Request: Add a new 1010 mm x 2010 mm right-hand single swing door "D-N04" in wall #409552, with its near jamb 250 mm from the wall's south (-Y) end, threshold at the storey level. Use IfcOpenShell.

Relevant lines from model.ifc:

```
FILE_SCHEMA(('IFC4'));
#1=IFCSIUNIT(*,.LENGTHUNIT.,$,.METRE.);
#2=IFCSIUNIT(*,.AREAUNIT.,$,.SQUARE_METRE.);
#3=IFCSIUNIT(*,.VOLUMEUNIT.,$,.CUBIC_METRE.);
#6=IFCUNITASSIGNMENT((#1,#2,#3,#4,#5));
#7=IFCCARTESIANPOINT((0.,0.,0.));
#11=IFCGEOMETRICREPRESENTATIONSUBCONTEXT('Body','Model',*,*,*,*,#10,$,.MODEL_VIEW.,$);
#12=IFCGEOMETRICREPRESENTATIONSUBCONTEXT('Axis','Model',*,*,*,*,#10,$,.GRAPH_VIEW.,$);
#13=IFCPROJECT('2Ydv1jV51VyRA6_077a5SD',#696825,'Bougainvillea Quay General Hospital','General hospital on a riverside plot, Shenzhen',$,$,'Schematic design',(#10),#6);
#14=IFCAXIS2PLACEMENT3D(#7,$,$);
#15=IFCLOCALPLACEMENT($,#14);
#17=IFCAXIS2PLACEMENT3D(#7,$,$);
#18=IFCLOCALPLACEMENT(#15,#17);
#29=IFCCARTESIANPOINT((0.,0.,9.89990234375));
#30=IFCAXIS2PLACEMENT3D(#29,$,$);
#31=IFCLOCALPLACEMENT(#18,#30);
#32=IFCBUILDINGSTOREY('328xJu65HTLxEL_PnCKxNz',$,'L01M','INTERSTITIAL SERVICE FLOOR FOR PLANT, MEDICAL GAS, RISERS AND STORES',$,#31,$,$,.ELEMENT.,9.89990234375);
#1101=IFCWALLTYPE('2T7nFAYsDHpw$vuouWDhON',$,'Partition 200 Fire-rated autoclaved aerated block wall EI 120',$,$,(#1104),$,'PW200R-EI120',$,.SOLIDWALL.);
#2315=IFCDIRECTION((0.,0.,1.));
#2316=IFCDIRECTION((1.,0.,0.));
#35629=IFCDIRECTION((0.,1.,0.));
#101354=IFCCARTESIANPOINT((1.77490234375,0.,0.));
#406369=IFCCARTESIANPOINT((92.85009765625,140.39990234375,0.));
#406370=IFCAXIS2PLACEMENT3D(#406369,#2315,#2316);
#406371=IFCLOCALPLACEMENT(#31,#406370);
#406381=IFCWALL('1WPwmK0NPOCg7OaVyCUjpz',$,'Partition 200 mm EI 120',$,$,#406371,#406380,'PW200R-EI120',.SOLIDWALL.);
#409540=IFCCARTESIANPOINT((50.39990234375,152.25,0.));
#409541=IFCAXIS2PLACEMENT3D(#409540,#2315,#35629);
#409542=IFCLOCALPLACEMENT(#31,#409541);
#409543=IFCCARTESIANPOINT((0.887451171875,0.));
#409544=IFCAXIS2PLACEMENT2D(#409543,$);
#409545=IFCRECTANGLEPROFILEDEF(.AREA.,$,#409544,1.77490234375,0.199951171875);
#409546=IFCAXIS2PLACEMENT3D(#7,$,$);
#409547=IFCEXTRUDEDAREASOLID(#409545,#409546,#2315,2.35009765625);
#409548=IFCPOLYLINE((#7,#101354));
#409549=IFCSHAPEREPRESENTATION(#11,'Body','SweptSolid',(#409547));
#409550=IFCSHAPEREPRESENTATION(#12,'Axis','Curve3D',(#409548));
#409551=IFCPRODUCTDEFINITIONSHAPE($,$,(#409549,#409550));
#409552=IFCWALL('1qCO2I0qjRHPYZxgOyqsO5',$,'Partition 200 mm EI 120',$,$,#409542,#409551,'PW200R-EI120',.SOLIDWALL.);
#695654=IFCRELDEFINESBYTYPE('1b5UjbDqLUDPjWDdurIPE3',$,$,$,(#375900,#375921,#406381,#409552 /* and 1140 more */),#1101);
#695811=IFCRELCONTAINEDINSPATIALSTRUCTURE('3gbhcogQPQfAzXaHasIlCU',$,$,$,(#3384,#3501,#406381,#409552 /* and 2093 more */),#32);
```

```python
import numpy as np
import ifcopenshell
import ifcopenshell.api.feature
import ifcopenshell.api.geometry
import ifcopenshell.api.root
import ifcopenshell.api.spatial
import ifcopenshell.geom
import ifcopenshell.util.element
import ifcopenshell.util.placement
import ifcopenshell.util.representation
import ifcopenshell.util.shape
import ifcopenshell.util.unit

model = ifcopenshell.open("model.ifc")
unit_scale = ifcopenshell.util.unit.calculate_unit_scale(model)
settings = ifcopenshell.geom.settings()


def volume(element):
    """Net volume in cubic metres, openings subtracted."""
    shape = ifcopenshell.geom.create_shape(settings, element)
    return ifcopenshell.util.shape.get_volume(shape.geometry)


wall = model.by_id(409552)
storey = ifcopenshell.util.element.get_container(wall, ifc_class="IfcBuildingStorey")
context = ifcopenshell.util.representation.get_context(model, "Model", "Body", "MODEL_VIEW")
before = volume(wall)

width, height, from_end, sill = 1.01, 2.01, 0.25, 0.0  # metres

# The wall runs along its own X axis, and the end named is its -X end.
wall_shape = ifcopenshell.geom.create_shape(settings, wall)
x, y, z = ifcopenshell.util.shape.get_vertices(wall_shape.geometry).T
start = x.min() + from_end
face, thickness = float(y.min()), float(y.max() - y.min())
wall_matrix = ifcopenshell.util.placement.get_local_placement(wall.ObjectPlacement)
level = ifcopenshell.util.placement.get_local_placement(storey.ObjectPlacement)[2, 3]


def in_wall(x, y):
    """Placement at x, y metres in the wall's axes, at sill height."""
    matrix = wall_matrix.copy()
    matrix[:, 3] = wall_matrix @ np.array([x / unit_scale, y / unit_scale, 0.0, 1.0])
    matrix[2, 3] = level + sill / unit_scale
    return matrix


# Opening: a box that overshoots both wall faces by 50 mm.
opening = ifcopenshell.api.root.create_entity(model, ifc_class="IfcOpeningElement", predefined_type="OPENING")
box = ifcopenshell.api.geometry.add_wall_representation(
    model, context=context, length=width, height=height, thickness=thickness + 0.1
)
ifcopenshell.api.geometry.assign_representation(model, product=opening, representation=box)
ifcopenshell.api.geometry.edit_object_placement(model, product=opening, matrix=in_wall(start, face - 0.05), is_si=False)
ifcopenshell.api.feature.add_feature(model, feature=opening, element=wall)

door = ifcopenshell.api.root.create_entity(model, ifc_class="IfcDoor", name="D-N04", predefined_type="DOOR")
door.OverallWidth, door.OverallHeight = width / unit_scale, height / unit_scale
door.OperationType = "SINGLE_SWING_RIGHT"
body = ifcopenshell.api.geometry.add_door_representation(
    model,
    context=context,
    overall_width=door.OverallWidth,
    overall_height=door.OverallHeight,
    operation_type="SINGLE_SWING_RIGHT",
    lining_properties={"LiningDepth": thickness / unit_scale, "ThresholdDepth": thickness / unit_scale},
)
ifcopenshell.api.geometry.assign_representation(model, product=door, representation=body)
ifcopenshell.api.spatial.assign_container(model, products=[door], relating_structure=storey)
ifcopenshell.api.feature.add_filling(model, opening=opening, element=door)

# The lining spans the wall, so the door starts at the wall face.
ifcopenshell.api.geometry.edit_object_placement(model, product=door, matrix=in_wall(start, face), is_si=False)

after = volume(wall)

print(f"wall volume {before:.3f} -> {after:.3f} m3")

model.write("model_rev.ifc")
```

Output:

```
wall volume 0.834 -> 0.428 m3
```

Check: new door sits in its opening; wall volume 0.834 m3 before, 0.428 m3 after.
